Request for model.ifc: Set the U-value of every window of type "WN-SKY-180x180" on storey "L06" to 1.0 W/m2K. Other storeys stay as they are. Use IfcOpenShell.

First a look at what the model holds.

```python
import ifcopenshell
import ifcopenshell.util.element

model = ifcopenshell.open("model.ifc")
print(model.schema)
storey = next(s for s in model.by_type("IfcBuildingStorey") if s.Name == "L06")
windows = [e for e in ifcopenshell.util.element.get_decomposition(storey) if e.is_a("IfcWindow")]
seen = {}
for e in windows:
    element_type = ifcopenshell.util.element.get_type(e)
    key = (element_type.Name if element_type != e and element_type else None, ifcopenshell.util.element.get_pset(e, "Pset_WindowCommon", "ThermalTransmittance"))
    seen[key] = seen.get(key, 0) + 1
for (name, value), count in sorted(seen.items(), key=str):
    print(count, "x", name, "|", value)
```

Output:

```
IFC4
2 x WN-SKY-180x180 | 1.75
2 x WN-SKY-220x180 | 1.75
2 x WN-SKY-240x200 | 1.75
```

```python
import ifcopenshell
import ifcopenshell.api.pset
import ifcopenshell.util.element

model = ifcopenshell.open("model.ifc")

storey = next(s for s in model.by_type("IfcBuildingStorey") if s.Name == "L06")
windows = [e for e in ifcopenshell.util.element.get_decomposition(storey) if e.is_a("IfcWindow")]

count = 0
for e in windows:
    element_type = ifcopenshell.util.element.get_type(e)
    if element_type in (None, e) or element_type.Name != "WN-SKY-180x180":
        continue
    # add_pset returns the element's existing set when there is one.
    pset = ifcopenshell.api.pset.add_pset(model, product=e, name="Pset_WindowCommon")
    ifcopenshell.api.pset.edit_pset(model, pset=pset, properties={"ThermalTransmittance": 1.0})
    count += 1

print(count, "windows updated")

model.write("model_v2.ifc")
```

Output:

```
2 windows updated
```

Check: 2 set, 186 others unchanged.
